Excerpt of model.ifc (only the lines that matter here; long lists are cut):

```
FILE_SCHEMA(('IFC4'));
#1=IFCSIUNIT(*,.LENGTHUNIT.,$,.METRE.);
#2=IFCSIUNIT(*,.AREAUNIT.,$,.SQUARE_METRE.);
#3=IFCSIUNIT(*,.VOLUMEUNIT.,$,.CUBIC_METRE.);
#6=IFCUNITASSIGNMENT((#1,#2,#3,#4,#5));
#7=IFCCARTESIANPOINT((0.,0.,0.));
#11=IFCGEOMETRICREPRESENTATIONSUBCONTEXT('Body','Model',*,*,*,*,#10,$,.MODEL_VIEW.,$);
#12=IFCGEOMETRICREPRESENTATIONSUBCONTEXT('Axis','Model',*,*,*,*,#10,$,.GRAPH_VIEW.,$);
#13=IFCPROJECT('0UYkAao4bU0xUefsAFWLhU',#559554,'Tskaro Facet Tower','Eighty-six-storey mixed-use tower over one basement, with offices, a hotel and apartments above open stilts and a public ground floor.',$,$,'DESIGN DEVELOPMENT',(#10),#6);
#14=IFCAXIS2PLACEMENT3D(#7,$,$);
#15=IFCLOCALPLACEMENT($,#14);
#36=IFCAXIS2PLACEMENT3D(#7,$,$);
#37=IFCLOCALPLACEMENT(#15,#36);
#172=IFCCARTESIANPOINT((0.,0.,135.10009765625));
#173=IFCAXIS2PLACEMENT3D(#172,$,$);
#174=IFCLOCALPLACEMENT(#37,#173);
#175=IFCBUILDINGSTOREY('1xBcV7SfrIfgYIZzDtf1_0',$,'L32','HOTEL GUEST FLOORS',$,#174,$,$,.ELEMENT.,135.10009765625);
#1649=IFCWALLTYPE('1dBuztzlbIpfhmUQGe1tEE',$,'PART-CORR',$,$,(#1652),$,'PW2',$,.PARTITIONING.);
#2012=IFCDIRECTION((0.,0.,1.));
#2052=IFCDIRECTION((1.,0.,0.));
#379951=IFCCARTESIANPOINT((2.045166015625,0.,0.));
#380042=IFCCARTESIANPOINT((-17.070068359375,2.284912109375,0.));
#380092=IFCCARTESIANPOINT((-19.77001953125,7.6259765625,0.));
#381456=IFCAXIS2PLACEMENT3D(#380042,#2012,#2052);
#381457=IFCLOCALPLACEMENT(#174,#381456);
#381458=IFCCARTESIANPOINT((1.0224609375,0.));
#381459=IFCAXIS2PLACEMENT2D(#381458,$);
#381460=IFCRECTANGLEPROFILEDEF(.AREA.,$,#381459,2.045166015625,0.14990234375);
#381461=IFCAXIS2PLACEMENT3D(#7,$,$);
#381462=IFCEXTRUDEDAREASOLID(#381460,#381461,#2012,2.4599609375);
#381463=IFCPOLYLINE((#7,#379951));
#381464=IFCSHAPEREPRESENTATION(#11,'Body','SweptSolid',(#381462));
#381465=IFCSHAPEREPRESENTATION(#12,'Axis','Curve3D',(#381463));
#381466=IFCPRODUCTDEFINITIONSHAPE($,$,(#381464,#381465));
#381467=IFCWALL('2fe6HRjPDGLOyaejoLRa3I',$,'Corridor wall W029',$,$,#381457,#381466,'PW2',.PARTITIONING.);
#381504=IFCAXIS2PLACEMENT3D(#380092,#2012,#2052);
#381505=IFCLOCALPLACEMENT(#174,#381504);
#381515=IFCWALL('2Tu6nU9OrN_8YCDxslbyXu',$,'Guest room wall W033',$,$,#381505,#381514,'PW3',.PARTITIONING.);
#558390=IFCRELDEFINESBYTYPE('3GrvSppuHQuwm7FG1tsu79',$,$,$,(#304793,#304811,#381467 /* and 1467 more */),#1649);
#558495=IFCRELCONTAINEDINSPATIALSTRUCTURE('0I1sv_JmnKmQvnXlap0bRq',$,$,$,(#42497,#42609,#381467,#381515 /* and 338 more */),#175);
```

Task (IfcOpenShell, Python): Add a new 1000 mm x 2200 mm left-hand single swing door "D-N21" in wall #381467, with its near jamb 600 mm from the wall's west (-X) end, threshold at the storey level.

```python
import numpy as np
import ifcopenshell
import ifcopenshell.api.feature
import ifcopenshell.api.geometry
import ifcopenshell.api.root
import ifcopenshell.api.spatial
import ifcopenshell.geom
import ifcopenshell.util.element
import ifcopenshell.util.placement
import ifcopenshell.util.representation
import ifcopenshell.util.shape
import ifcopenshell.util.unit

model = ifcopenshell.open("model.ifc")
unit_scale = ifcopenshell.util.unit.calculate_unit_scale(model)
settings = ifcopenshell.geom.settings()


def volume(element):
    """Net volume in cubic metres, openings subtracted."""
    shape = ifcopenshell.geom.create_shape(settings, element)
    return ifcopenshell.util.shape.get_volume(shape.geometry)


wall = model.by_guid("2fe6HRjPDGLOyaejoLRa3I")
storey = ifcopenshell.util.element.get_container(wall, ifc_class="IfcBuildingStorey")
context = ifcopenshell.util.representation.get_context(model, "Model", "Body", "MODEL_VIEW")
before = volume(wall)

width, height, from_end, sill = 1, 2.2, 0.6, 0.0  # metres

# The wall runs along its own X axis, and the end named is its -X end.
wall_shape = ifcopenshell.geom.create_shape(settings, wall)
x, y, z = ifcopenshell.util.shape.get_vertices(wall_shape.geometry).T
start = x.min() + from_end
face, thickness = float(y.min()), float(y.max() - y.min())
wall_matrix = ifcopenshell.util.placement.get_local_placement(wall.ObjectPlacement)
level = ifcopenshell.util.placement.get_local_placement(storey.ObjectPlacement)[2, 3]


def in_wall(x, y):
    """Placement at x, y metres in the wall's axes, at sill height."""
    matrix = wall_matrix.copy()
    matrix[:, 3] = wall_matrix @ np.array([x / unit_scale, y / unit_scale, 0.0, 1.0])
    matrix[2, 3] = level + sill / unit_scale
    return matrix


# Opening: a box that overshoots both wall faces by 50 mm.
opening = ifcopenshell.api.root.create_entity(model, ifc_class="IfcOpeningElement", predefined_type="OPENING")
box = ifcopenshell.api.geometry.add_wall_representation(
    model, context=context, length=width, height=height, thickness=thickness + 0.1
)
ifcopenshell.api.geometry.assign_representation(model, product=opening, representation=box)
ifcopenshell.api.geometry.edit_object_placement(model, product=opening, matrix=in_wall(start, face - 0.05), is_si=False)
ifcopenshell.api.feature.add_feature(model, feature=opening, element=wall)

door = ifcopenshell.api.root.create_entity(model, ifc_class="IfcDoor", name="D-N21", predefined_type="DOOR")
door.OverallWidth, door.OverallHeight = width / unit_scale, height / unit_scale
door.OperationType = "SINGLE_SWING_LEFT"
body = ifcopenshell.api.geometry.add_door_representation(
    model,
    context=context,
    overall_width=door.OverallWidth,
    overall_height=door.OverallHeight,
    operation_type="SINGLE_SWING_LEFT",
    lining_properties={"LiningDepth": thickness / unit_scale, "ThresholdDepth": thickness / unit_scale},
)
ifcopenshell.api.geometry.assign_representation(model, product=door, representation=body)
ifcopenshell.api.spatial.assign_container(model, products=[door], relating_structure=storey)
ifcopenshell.api.feature.add_filling(model, opening=opening, element=door)

# The lining spans the wall, so the door starts at the wall face.
ifcopenshell.api.geometry.edit_object_placement(model, product=door, matrix=in_wall(start, face), is_si=False)

after = volume(wall)

print(f"wall volume {before:.3f} -> {after:.3f} m3")

model.write("model_edited.ifc")
```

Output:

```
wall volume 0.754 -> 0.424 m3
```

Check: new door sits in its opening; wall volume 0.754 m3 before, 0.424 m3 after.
